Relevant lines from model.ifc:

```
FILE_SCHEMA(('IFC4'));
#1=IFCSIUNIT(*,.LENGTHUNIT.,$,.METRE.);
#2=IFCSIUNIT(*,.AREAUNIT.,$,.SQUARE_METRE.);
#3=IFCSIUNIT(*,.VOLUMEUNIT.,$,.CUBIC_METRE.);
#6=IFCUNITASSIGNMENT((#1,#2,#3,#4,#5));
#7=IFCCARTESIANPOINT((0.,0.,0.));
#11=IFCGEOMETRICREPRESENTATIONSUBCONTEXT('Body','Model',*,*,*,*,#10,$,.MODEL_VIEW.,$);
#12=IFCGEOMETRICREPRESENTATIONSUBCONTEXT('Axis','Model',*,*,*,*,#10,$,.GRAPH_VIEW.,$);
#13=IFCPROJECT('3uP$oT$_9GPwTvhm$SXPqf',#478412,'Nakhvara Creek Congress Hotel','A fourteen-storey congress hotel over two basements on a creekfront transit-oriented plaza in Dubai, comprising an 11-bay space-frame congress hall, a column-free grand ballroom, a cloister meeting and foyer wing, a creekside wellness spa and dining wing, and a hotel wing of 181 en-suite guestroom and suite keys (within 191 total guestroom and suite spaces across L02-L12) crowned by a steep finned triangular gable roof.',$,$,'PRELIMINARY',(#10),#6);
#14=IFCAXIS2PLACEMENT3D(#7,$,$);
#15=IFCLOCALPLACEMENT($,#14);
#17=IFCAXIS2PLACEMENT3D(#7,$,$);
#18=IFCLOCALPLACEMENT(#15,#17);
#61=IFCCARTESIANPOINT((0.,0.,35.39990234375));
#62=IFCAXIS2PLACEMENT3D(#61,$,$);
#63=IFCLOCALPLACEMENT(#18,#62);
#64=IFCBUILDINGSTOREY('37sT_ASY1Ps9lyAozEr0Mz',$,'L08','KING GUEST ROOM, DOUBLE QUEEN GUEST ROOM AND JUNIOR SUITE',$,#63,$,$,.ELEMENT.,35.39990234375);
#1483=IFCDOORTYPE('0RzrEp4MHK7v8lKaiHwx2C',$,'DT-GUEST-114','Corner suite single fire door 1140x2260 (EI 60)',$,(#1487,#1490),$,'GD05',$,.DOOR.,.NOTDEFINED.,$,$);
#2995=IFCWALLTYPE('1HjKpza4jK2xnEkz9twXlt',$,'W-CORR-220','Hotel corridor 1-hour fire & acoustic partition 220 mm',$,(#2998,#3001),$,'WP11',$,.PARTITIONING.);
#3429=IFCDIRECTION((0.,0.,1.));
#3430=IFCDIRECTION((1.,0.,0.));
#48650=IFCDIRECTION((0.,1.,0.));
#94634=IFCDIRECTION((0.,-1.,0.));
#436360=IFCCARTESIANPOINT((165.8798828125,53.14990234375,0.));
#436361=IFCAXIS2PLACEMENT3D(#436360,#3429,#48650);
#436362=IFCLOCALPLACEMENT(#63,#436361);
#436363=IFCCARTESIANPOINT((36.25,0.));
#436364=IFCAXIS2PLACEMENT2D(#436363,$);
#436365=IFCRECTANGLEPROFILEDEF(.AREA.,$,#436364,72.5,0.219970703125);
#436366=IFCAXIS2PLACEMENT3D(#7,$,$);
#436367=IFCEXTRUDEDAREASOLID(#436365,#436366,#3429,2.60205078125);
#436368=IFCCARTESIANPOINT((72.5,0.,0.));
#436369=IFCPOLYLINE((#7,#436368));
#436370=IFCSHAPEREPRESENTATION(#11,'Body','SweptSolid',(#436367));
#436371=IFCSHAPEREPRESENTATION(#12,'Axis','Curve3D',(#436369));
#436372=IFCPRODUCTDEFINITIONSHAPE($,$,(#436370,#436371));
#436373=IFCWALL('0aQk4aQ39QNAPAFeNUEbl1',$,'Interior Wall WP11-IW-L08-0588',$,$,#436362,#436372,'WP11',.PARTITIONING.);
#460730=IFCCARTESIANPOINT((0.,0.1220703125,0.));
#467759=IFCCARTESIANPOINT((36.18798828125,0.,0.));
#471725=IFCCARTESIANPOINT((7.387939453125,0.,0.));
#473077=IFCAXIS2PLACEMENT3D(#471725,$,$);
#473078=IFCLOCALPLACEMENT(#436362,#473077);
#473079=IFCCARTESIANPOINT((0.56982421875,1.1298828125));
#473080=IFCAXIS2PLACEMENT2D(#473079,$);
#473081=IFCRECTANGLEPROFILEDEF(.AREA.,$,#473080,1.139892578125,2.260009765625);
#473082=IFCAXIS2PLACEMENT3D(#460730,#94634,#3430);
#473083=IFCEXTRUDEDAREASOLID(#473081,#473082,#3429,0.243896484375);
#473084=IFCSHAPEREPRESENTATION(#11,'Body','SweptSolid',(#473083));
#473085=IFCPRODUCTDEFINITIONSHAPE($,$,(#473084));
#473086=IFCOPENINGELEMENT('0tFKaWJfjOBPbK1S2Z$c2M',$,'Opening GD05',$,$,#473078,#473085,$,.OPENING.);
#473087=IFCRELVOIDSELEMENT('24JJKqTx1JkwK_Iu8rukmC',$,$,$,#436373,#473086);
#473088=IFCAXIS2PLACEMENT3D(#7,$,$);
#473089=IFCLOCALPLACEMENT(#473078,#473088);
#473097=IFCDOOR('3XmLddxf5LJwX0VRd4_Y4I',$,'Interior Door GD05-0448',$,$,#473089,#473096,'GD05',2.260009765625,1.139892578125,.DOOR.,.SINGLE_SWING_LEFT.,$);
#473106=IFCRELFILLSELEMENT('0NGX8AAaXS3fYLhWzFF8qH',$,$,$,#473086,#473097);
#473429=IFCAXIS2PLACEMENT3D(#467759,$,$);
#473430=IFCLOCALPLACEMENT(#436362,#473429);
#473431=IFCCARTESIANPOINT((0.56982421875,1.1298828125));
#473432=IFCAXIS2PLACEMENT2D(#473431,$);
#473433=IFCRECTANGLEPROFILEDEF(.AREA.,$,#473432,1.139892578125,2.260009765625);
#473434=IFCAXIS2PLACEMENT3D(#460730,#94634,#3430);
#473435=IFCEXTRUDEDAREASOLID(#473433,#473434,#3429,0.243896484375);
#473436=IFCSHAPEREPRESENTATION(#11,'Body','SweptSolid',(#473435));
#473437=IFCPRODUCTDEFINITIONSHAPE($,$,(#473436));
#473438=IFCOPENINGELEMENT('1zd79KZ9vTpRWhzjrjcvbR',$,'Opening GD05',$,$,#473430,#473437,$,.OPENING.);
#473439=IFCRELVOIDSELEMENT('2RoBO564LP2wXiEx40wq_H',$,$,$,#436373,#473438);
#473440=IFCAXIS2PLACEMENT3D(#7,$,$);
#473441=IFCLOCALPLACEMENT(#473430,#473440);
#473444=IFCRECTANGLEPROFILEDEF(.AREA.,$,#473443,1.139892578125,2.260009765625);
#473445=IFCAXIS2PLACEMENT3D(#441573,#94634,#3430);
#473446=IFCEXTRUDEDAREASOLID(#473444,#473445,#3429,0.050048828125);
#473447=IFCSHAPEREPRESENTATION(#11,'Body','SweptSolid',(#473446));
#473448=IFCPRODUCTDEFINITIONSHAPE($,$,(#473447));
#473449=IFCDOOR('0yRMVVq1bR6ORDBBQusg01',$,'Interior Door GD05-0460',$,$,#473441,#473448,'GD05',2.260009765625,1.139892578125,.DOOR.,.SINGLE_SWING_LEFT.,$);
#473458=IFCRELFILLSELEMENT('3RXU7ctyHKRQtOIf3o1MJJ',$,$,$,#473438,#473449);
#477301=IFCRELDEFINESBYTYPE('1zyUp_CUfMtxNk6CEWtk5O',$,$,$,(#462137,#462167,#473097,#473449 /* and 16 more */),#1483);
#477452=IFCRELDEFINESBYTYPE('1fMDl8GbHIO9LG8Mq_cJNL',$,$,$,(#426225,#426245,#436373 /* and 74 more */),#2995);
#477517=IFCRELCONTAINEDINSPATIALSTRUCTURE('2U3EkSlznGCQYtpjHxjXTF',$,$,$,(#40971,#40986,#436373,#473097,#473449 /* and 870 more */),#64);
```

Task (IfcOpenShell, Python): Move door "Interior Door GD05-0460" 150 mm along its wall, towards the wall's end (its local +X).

```python
import ifcopenshell
import ifcopenshell.api.geometry
import ifcopenshell.util.placement
import ifcopenshell.util.unit

model = ifcopenshell.open("model.ifc")
unit_scale = ifcopenshell.util.unit.calculate_unit_scale(model)

door = model.by_guid("0yRMVVq1bR6ORDBBQusg01")
opening = door.FillsVoids[0].RelatingOpeningElement
wall = opening.VoidsElements[0].RelatingBuildingElement

wall_matrix = ifcopenshell.util.placement.get_local_placement(wall.ObjectPlacement)
shift = wall_matrix[:3, 0] * 0.15 / unit_scale
before = ifcopenshell.util.placement.get_local_placement(door.ObjectPlacement)[:3, 3].copy()

# The door is placed relative to its opening, so it follows when the opening moves.
matrix = ifcopenshell.util.placement.get_local_placement(opening.ObjectPlacement)
matrix[:3, 3] += shift
ifcopenshell.api.geometry.edit_object_placement(
    model, product=opening, matrix=matrix, is_si=False, should_transform_children=True
)

after = ifcopenshell.util.placement.get_local_placement(door.ObjectPlacement)[:3, 3]
print("door moved by", (after - before).round(3) + 0.0)

model.write("model_rev.ifc")
```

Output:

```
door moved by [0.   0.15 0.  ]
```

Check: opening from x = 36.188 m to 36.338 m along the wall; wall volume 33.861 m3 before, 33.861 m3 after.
